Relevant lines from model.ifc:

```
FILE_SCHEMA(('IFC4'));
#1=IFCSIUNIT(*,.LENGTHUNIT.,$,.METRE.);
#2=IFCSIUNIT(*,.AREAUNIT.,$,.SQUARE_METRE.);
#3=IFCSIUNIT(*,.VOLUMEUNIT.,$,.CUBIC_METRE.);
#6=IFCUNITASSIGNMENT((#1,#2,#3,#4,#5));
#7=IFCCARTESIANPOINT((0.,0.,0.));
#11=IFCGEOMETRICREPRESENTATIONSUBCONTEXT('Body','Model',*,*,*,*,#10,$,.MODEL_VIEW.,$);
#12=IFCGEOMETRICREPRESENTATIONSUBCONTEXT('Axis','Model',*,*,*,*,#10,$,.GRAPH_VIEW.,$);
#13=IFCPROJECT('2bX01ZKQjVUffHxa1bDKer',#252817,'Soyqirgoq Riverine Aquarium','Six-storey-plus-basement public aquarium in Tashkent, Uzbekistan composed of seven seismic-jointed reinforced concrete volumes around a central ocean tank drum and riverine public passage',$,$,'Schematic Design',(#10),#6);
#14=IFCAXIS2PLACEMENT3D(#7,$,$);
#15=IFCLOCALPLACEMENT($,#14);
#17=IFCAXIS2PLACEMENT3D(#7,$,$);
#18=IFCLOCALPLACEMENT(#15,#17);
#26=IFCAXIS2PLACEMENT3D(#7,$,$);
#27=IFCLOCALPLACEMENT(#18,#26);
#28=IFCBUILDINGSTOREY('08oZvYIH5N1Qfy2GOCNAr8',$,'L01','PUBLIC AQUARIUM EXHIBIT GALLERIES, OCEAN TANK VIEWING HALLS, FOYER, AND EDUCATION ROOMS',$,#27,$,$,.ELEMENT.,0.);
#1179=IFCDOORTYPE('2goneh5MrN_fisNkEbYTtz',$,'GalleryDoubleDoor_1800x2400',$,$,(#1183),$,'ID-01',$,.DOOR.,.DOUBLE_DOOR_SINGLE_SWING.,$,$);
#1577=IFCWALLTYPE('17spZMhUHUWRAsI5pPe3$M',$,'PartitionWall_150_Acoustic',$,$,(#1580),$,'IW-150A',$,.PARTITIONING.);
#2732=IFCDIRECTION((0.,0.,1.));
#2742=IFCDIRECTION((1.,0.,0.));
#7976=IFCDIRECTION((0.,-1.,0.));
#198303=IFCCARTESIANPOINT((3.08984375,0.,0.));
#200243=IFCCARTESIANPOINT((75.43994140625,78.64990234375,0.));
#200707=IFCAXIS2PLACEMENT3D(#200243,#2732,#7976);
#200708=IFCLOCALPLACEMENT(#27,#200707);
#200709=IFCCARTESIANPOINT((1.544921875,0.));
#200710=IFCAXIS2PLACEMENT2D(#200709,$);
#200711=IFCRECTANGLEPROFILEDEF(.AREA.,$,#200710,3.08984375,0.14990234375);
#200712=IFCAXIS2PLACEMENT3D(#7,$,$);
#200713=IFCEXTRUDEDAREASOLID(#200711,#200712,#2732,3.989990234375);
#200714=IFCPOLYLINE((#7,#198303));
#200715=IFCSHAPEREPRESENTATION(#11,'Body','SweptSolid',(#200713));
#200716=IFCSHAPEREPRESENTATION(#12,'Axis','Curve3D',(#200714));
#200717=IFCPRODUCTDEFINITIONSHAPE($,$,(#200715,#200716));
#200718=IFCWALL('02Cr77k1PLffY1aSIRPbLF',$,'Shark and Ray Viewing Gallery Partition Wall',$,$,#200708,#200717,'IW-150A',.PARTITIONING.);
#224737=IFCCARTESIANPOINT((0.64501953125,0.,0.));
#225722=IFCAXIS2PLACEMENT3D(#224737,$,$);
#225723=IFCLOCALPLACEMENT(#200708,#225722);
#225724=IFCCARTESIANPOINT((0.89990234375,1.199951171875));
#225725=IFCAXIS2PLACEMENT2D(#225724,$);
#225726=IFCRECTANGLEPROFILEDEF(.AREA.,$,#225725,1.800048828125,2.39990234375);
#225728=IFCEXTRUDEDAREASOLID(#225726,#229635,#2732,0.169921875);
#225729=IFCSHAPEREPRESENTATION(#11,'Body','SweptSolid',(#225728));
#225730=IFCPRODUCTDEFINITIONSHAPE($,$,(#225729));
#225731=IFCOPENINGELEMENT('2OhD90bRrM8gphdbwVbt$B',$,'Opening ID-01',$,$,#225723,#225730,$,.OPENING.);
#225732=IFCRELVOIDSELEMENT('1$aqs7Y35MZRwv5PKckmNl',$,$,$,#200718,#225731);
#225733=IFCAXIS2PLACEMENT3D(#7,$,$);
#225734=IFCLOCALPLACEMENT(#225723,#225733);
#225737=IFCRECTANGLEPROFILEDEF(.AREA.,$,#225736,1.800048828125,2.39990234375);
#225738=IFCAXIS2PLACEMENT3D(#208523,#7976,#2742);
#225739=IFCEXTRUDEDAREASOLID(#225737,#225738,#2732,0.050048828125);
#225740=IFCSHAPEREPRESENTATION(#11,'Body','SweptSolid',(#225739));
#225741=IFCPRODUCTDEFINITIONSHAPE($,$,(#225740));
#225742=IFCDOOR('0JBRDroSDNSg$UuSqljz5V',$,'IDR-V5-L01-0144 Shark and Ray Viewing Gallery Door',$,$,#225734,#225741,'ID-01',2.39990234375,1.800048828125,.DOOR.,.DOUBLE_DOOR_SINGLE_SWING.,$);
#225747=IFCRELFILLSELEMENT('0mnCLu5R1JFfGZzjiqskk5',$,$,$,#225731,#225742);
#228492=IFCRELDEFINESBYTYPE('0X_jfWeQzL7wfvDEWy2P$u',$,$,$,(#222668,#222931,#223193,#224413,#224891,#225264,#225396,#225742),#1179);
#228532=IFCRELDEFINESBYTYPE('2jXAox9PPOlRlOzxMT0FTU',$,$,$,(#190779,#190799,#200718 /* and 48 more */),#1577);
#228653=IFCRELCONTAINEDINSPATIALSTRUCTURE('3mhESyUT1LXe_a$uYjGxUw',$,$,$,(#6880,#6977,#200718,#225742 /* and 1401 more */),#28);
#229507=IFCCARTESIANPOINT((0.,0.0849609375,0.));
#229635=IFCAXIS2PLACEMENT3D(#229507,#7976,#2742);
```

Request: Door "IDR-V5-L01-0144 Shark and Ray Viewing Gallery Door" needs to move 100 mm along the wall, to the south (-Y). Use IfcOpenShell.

```python
import ifcopenshell
import ifcopenshell.api.geometry
import ifcopenshell.util.placement
import ifcopenshell.util.unit

model = ifcopenshell.open("model.ifc")
unit_scale = ifcopenshell.util.unit.calculate_unit_scale(model)

door = model.by_id(225742)
opening = door.FillsVoids[0].RelatingOpeningElement
wall = opening.VoidsElements[0].RelatingBuildingElement

wall_matrix = ifcopenshell.util.placement.get_local_placement(wall.ObjectPlacement)
shift = wall_matrix[:3, 0] * 0.1 / unit_scale
before = ifcopenshell.util.placement.get_local_placement(door.ObjectPlacement)[:3, 3].copy()

# The door is placed relative to its opening, so it follows when the opening moves.
matrix = ifcopenshell.util.placement.get_local_placement(opening.ObjectPlacement)
matrix[:3, 3] += shift
ifcopenshell.api.geometry.edit_object_placement(
    model, product=opening, matrix=matrix, is_si=False, should_transform_children=True
)

after = ifcopenshell.util.placement.get_local_placement(door.ObjectPlacement)[:3, 3]
print("door moved by", (after - before).round(3) + 0.0)

model.write("model-out.ifc")
```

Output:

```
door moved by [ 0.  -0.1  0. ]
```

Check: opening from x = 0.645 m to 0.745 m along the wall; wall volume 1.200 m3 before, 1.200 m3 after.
